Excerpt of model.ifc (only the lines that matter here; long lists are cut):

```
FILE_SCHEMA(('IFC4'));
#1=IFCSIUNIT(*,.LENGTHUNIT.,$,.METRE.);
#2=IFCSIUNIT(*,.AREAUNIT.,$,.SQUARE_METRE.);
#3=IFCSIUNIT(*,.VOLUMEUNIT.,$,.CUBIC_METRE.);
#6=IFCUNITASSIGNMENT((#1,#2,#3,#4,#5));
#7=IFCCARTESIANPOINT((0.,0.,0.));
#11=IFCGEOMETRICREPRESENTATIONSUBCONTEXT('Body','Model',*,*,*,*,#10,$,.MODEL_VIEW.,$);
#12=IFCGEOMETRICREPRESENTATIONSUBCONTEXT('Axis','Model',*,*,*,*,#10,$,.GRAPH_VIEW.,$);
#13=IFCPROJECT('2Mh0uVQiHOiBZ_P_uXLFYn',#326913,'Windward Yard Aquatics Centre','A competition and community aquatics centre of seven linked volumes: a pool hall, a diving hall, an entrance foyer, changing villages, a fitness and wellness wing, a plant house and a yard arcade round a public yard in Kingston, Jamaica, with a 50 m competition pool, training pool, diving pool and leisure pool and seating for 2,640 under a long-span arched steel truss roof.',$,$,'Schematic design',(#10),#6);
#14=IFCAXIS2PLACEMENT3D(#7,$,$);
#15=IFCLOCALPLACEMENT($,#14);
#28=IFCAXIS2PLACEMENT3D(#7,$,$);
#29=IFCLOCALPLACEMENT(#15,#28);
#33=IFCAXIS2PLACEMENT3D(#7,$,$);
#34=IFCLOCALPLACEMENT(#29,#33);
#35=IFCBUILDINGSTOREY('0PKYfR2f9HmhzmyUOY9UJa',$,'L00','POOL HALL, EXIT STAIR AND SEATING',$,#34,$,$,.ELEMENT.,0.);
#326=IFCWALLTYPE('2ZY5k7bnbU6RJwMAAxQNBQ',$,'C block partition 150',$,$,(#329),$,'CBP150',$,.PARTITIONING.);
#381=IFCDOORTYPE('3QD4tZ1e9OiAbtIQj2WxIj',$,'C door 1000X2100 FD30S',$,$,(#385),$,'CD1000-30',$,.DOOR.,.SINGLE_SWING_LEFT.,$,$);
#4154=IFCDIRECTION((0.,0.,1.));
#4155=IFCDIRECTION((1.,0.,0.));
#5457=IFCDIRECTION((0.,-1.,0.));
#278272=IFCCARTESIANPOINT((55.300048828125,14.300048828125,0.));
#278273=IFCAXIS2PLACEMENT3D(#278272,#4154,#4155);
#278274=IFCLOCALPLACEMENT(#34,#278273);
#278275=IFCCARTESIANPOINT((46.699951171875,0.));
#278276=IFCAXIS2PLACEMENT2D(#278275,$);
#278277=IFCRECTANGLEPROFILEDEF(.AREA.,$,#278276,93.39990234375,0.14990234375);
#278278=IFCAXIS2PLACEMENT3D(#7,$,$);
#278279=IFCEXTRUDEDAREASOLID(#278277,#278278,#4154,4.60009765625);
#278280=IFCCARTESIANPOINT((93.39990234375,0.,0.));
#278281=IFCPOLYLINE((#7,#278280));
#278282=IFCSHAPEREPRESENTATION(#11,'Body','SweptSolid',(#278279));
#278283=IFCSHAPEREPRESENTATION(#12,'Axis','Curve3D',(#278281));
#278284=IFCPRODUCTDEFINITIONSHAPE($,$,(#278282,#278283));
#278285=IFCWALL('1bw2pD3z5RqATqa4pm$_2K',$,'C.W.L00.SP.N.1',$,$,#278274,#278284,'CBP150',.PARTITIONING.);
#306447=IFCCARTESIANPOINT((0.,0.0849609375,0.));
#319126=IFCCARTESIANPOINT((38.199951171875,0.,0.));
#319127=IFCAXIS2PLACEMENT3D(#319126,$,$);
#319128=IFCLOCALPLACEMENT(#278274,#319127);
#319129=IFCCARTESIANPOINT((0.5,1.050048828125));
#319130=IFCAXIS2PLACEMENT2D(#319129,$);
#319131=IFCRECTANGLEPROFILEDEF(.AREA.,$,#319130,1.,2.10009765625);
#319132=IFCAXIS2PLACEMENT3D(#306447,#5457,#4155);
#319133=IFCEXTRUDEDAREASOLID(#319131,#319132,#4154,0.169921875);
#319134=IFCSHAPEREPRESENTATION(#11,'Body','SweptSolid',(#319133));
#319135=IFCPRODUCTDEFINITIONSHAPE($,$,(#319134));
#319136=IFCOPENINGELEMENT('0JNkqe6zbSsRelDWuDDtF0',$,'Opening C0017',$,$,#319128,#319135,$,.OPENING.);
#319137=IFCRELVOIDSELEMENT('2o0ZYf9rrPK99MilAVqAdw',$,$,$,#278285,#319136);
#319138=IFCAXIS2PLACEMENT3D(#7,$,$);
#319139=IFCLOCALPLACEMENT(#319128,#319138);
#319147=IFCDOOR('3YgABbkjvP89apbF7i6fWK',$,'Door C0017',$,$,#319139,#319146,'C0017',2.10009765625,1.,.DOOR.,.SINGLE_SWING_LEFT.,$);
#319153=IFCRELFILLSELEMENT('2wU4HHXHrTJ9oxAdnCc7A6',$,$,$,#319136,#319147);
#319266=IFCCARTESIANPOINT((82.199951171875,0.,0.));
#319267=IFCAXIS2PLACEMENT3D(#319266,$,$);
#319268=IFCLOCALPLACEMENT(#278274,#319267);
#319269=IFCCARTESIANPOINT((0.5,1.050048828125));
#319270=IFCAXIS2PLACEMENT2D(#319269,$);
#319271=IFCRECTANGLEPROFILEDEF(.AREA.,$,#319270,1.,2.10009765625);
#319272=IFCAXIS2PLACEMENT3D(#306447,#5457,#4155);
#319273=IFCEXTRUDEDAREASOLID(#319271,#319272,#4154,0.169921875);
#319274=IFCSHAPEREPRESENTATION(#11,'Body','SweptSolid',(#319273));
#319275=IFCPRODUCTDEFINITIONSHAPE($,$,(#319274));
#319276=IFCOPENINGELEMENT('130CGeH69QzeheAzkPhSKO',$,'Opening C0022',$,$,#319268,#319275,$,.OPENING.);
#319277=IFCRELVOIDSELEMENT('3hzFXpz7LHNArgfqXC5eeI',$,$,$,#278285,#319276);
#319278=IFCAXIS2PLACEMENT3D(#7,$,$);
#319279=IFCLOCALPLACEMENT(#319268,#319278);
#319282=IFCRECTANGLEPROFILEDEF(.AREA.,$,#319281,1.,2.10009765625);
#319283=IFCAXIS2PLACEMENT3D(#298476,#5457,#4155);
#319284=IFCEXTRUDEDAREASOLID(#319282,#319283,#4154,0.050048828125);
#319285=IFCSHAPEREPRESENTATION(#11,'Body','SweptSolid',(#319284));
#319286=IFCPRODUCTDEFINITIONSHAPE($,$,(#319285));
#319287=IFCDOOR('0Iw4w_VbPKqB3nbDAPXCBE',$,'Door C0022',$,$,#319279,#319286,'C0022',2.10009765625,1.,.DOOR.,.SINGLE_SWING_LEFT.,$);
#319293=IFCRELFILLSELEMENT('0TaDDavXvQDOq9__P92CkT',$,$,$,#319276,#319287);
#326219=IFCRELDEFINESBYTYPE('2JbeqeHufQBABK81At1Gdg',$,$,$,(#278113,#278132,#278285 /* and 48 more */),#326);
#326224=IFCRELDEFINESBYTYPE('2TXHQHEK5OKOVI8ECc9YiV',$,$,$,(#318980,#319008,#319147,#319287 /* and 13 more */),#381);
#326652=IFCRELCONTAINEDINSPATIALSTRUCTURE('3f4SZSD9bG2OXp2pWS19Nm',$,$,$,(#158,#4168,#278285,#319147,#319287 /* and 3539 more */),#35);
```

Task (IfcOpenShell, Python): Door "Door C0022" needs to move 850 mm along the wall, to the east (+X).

```python
import ifcopenshell
import ifcopenshell.api.geometry
import ifcopenshell.util.placement
import ifcopenshell.util.unit

model = ifcopenshell.open("model.ifc")
unit_scale = ifcopenshell.util.unit.calculate_unit_scale(model)

door = model.by_guid("0Iw4w_VbPKqB3nbDAPXCBE")
opening = door.FillsVoids[0].RelatingOpeningElement
wall = opening.VoidsElements[0].RelatingBuildingElement

wall_matrix = ifcopenshell.util.placement.get_local_placement(wall.ObjectPlacement)
shift = wall_matrix[:3, 0] * 0.85 / unit_scale
before = ifcopenshell.util.placement.get_local_placement(door.ObjectPlacement)[:3, 3].copy()

# The door is placed relative to its opening, so it follows when the opening moves.
matrix = ifcopenshell.util.placement.get_local_placement(opening.ObjectPlacement)
matrix[:3, 3] += shift
ifcopenshell.api.geometry.edit_object_placement(
    model, product=opening, matrix=matrix, is_si=False, should_transform_children=True
)

after = ifcopenshell.util.placement.get_local_placement(door.ObjectPlacement)[:3, 3]
print("door moved by", (after - before).round(3) + 0.0)

model.write("model_v2.ifc")
```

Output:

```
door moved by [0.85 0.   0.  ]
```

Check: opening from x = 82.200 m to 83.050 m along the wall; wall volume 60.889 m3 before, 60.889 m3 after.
